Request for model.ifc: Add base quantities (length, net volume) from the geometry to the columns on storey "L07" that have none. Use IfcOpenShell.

First a look at what the model holds.

```python
import ifcopenshell
import ifcopenshell.util.element
import ifcopenshell.util.unit

model = ifcopenshell.open("model.ifc")
print(model.schema)
for unit_type in ("LENGTHUNIT", "AREAUNIT", "VOLUMEUNIT"):
    print(unit_type, ifcopenshell.util.unit.calculate_unit_scale(model, unit_type))
storey = next(s for s in model.by_type("IfcBuildingStorey") if s.Name == "L07")
columns = [e for e in ifcopenshell.util.element.get_decomposition(storey) if e.is_a("IfcColumn")]
for e in sorted(columns, key=lambda e: e.id()):
    print(e.id(), e.is_a(), e.Name, list(ifcopenshell.util.element.get_psets(e, qtos_only=True)), sep=" | ")
```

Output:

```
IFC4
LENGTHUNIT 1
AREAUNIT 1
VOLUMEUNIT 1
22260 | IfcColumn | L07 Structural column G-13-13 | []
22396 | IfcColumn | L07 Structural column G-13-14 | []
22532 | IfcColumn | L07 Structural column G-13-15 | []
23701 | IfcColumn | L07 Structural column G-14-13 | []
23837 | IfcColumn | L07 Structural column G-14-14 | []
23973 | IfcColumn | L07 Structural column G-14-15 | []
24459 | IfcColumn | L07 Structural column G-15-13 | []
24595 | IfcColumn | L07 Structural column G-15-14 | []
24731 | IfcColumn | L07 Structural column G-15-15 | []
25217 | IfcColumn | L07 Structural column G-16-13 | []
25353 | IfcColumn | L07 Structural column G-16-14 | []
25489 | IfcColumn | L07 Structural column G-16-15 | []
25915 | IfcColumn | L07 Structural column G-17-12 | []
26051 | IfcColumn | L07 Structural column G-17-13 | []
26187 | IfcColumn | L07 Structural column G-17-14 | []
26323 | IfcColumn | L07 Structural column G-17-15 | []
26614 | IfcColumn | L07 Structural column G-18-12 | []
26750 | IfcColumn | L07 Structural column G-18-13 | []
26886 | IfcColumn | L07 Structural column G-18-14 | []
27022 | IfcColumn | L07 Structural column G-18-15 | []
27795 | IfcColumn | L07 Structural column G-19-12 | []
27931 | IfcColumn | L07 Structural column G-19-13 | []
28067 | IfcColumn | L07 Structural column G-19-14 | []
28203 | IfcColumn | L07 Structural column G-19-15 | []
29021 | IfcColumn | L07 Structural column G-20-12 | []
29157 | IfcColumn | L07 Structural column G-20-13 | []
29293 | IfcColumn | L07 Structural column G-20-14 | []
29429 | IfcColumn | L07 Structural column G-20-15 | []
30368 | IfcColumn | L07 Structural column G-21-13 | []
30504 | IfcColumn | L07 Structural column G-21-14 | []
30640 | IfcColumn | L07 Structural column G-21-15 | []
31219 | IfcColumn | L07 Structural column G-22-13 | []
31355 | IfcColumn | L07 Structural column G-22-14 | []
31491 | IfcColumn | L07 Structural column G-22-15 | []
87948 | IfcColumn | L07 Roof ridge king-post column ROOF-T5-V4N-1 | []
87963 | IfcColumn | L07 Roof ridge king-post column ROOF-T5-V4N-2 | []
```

```python
import ifcopenshell
import ifcopenshell.api.pset
import ifcopenshell.geom
import ifcopenshell.util.element
import ifcopenshell.util.shape
import ifcopenshell.util.unit

model = ifcopenshell.open("model.ifc")
unit_scale = ifcopenshell.util.unit.calculate_unit_scale(model)
volume_scale = ifcopenshell.util.unit.calculate_unit_scale(model, "VOLUMEUNIT")
settings = ifcopenshell.geom.settings()

storey = next(s for s in model.by_type("IfcBuildingStorey") if s.Name == "L07")
columns = [e for e in ifcopenshell.util.element.get_decomposition(storey) if e.is_a("IfcColumn")]

for e in sorted(columns, key=lambda e: e.id()):
    if ifcopenshell.util.element.get_psets(e, qtos_only=True, should_inherit=False):
        continue
    # Geometry comes back in metres, in the element's own axes.
    shape = ifcopenshell.geom.create_shape(settings, e)
    values = {
        "Length": ifcopenshell.util.shape.get_z(shape.geometry) / unit_scale,
        "NetVolume": ifcopenshell.util.shape.get_volume(shape.geometry) / volume_scale,
    }
    qto = ifcopenshell.api.pset.add_qto(model, product=e, name="Qto_ColumnBaseQuantities")
    ifcopenshell.api.pset.edit_qto(model, qto=qto, properties=values)
    print(e.id(), {k: round(v, 3) for k, v in values.items()})

model.write("model_v2.ifc")
```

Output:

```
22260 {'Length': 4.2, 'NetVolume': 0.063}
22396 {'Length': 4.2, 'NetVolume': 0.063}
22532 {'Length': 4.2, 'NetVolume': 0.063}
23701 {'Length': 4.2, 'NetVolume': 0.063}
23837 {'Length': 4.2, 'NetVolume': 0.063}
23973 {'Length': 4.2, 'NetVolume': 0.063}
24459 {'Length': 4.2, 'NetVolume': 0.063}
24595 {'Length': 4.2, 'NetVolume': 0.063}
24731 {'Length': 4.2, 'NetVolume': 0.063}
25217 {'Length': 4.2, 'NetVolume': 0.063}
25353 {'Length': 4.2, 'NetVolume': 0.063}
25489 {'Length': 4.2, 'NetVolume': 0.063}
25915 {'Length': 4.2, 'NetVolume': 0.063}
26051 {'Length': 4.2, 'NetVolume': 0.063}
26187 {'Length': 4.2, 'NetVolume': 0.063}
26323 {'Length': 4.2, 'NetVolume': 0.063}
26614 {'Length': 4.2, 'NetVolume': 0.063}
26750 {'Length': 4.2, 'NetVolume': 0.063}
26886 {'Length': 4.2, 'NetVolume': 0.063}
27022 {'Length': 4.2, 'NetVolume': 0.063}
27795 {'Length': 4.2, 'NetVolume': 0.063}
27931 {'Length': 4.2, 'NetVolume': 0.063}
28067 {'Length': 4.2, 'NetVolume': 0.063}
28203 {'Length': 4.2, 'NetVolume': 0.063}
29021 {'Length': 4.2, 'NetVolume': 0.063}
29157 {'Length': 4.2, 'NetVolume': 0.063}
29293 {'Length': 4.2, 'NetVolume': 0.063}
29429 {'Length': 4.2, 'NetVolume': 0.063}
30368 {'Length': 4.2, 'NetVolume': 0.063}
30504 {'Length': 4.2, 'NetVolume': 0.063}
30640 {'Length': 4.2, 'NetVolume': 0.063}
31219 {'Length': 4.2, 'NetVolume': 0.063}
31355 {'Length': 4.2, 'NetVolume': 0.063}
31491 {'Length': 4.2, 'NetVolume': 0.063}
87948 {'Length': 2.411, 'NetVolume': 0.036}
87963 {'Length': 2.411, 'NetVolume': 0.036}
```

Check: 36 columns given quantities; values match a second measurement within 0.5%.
